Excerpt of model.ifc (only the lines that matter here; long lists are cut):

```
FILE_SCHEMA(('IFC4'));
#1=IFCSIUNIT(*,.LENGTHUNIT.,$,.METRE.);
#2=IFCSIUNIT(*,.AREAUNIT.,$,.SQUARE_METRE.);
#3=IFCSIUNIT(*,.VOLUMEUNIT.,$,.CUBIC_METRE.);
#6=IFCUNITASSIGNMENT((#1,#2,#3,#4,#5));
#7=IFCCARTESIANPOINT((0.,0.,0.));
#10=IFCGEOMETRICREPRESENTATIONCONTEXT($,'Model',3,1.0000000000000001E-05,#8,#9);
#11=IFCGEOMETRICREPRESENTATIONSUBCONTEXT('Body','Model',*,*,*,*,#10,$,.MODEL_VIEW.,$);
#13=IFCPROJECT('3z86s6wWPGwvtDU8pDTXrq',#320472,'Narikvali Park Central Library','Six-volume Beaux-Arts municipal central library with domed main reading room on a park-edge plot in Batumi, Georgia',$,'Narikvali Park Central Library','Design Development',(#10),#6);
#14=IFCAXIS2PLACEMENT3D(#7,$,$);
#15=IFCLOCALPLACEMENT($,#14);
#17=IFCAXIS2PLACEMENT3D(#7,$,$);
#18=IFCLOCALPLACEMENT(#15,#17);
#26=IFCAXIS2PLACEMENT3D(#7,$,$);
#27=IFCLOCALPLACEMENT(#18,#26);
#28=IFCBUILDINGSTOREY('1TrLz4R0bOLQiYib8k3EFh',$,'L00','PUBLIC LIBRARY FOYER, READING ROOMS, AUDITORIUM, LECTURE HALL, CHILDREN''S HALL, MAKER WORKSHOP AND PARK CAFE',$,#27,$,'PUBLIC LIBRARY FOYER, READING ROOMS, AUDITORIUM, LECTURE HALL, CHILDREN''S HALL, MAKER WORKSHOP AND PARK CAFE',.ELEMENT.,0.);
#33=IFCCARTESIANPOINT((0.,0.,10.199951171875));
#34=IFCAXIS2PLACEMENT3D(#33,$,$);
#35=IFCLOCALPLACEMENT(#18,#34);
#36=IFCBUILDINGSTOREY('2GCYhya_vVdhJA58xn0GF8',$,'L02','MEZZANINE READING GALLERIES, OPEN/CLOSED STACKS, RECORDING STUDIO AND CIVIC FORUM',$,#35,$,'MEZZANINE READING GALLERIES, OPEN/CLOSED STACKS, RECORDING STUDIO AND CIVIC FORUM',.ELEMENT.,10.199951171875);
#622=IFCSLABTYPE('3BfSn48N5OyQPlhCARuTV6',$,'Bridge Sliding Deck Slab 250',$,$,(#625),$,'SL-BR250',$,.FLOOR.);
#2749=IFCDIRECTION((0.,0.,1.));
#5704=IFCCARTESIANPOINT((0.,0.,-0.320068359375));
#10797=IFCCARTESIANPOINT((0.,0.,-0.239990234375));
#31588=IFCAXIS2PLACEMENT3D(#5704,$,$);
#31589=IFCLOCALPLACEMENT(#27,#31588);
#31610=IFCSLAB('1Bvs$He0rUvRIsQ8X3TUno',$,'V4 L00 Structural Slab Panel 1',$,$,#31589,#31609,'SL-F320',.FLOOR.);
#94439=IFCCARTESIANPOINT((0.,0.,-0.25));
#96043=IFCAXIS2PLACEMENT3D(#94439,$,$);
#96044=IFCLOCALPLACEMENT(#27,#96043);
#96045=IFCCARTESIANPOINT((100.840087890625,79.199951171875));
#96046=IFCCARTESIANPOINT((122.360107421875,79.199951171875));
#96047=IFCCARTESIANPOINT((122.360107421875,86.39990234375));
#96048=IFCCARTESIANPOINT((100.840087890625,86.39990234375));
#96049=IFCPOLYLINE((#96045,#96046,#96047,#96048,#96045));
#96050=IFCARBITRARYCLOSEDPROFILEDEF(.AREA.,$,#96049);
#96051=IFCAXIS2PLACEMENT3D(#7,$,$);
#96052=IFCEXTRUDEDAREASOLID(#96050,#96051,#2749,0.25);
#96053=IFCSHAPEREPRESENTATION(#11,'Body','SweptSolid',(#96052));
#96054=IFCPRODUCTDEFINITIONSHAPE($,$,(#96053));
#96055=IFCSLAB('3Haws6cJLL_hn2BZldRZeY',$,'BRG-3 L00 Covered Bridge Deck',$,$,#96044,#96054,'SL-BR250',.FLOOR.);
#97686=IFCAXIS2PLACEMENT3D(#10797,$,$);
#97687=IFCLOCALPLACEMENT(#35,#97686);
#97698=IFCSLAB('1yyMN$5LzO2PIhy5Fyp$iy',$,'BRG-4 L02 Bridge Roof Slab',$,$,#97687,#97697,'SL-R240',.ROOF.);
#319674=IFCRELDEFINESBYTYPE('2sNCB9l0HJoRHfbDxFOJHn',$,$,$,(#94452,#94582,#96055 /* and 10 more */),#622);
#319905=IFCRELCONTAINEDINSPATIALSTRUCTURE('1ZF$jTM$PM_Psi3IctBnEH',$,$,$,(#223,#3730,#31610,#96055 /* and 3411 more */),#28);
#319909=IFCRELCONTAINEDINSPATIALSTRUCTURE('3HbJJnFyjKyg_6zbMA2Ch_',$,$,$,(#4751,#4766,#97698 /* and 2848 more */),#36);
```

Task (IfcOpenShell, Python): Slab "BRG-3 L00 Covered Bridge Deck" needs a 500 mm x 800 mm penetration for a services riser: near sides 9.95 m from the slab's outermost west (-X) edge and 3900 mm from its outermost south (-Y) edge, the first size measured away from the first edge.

```python
import numpy as np
import ifcopenshell
import ifcopenshell.api.feature
import ifcopenshell.api.geometry
import ifcopenshell.api.root
import ifcopenshell.geom
import ifcopenshell.util.placement
import ifcopenshell.util.representation
import ifcopenshell.util.shape
import ifcopenshell.util.unit

model = ifcopenshell.open("model.ifc")
unit_scale = ifcopenshell.util.unit.calculate_unit_scale(model)
settings = ifcopenshell.geom.settings()


def volume(element):
    """Net volume in cubic metres, openings subtracted."""
    shape = ifcopenshell.geom.create_shape(settings, element)
    return ifcopenshell.util.shape.get_volume(shape.geometry)


slab = model.by_guid("3Haws6cJLL_hn2BZldRZeY")
before = volume(slab)

# Extent in the slab's own axes, in metres. The edges named are its -X and -Y sides.
slab_shape = ifcopenshell.geom.create_shape(settings, slab)
vertices = ifcopenshell.util.shape.get_vertices(slab_shape.geometry)
x_min, y_min, bottom = vertices.min(axis=0)
top = vertices[:, 2].max()

opening = ifcopenshell.api.root.create_entity(model, ifc_class="IfcOpeningElement", name="Services riser opening", predefined_type="OPENING")
context = ifcopenshell.util.representation.get_context(model, "Model", "Body", "MODEL_VIEW")
width, depth = 0.5, 0.8
outline = [(0.0, 0.0), (width, 0.0), (width, depth), (0.0, depth), (0.0, 0.0)]
# Overshoot both faces by 50 mm so the cut is clean.
shape = ifcopenshell.api.geometry.add_slab_representation(
    model, context=context, depth=top - bottom + 0.1, polyline=outline
)
ifcopenshell.api.geometry.assign_representation(model, product=opening, representation=shape)

matrix = ifcopenshell.util.placement.get_local_placement(slab.ObjectPlacement)
matrix[:, 3] = matrix @ np.append(np.array([x_min + 9.95, y_min + 3.9, bottom - 0.05]) / unit_scale, 1.0)
ifcopenshell.api.geometry.edit_object_placement(model, product=opening, matrix=matrix, is_si=False)
ifcopenshell.api.feature.add_feature(model, feature=opening, element=slab)

after = volume(slab)

print(f"slab volume {before:.3f} -> {after:.3f} m3")

model.write("model_rev.ifc")
```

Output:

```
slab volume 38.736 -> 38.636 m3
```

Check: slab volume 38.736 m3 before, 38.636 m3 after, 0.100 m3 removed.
